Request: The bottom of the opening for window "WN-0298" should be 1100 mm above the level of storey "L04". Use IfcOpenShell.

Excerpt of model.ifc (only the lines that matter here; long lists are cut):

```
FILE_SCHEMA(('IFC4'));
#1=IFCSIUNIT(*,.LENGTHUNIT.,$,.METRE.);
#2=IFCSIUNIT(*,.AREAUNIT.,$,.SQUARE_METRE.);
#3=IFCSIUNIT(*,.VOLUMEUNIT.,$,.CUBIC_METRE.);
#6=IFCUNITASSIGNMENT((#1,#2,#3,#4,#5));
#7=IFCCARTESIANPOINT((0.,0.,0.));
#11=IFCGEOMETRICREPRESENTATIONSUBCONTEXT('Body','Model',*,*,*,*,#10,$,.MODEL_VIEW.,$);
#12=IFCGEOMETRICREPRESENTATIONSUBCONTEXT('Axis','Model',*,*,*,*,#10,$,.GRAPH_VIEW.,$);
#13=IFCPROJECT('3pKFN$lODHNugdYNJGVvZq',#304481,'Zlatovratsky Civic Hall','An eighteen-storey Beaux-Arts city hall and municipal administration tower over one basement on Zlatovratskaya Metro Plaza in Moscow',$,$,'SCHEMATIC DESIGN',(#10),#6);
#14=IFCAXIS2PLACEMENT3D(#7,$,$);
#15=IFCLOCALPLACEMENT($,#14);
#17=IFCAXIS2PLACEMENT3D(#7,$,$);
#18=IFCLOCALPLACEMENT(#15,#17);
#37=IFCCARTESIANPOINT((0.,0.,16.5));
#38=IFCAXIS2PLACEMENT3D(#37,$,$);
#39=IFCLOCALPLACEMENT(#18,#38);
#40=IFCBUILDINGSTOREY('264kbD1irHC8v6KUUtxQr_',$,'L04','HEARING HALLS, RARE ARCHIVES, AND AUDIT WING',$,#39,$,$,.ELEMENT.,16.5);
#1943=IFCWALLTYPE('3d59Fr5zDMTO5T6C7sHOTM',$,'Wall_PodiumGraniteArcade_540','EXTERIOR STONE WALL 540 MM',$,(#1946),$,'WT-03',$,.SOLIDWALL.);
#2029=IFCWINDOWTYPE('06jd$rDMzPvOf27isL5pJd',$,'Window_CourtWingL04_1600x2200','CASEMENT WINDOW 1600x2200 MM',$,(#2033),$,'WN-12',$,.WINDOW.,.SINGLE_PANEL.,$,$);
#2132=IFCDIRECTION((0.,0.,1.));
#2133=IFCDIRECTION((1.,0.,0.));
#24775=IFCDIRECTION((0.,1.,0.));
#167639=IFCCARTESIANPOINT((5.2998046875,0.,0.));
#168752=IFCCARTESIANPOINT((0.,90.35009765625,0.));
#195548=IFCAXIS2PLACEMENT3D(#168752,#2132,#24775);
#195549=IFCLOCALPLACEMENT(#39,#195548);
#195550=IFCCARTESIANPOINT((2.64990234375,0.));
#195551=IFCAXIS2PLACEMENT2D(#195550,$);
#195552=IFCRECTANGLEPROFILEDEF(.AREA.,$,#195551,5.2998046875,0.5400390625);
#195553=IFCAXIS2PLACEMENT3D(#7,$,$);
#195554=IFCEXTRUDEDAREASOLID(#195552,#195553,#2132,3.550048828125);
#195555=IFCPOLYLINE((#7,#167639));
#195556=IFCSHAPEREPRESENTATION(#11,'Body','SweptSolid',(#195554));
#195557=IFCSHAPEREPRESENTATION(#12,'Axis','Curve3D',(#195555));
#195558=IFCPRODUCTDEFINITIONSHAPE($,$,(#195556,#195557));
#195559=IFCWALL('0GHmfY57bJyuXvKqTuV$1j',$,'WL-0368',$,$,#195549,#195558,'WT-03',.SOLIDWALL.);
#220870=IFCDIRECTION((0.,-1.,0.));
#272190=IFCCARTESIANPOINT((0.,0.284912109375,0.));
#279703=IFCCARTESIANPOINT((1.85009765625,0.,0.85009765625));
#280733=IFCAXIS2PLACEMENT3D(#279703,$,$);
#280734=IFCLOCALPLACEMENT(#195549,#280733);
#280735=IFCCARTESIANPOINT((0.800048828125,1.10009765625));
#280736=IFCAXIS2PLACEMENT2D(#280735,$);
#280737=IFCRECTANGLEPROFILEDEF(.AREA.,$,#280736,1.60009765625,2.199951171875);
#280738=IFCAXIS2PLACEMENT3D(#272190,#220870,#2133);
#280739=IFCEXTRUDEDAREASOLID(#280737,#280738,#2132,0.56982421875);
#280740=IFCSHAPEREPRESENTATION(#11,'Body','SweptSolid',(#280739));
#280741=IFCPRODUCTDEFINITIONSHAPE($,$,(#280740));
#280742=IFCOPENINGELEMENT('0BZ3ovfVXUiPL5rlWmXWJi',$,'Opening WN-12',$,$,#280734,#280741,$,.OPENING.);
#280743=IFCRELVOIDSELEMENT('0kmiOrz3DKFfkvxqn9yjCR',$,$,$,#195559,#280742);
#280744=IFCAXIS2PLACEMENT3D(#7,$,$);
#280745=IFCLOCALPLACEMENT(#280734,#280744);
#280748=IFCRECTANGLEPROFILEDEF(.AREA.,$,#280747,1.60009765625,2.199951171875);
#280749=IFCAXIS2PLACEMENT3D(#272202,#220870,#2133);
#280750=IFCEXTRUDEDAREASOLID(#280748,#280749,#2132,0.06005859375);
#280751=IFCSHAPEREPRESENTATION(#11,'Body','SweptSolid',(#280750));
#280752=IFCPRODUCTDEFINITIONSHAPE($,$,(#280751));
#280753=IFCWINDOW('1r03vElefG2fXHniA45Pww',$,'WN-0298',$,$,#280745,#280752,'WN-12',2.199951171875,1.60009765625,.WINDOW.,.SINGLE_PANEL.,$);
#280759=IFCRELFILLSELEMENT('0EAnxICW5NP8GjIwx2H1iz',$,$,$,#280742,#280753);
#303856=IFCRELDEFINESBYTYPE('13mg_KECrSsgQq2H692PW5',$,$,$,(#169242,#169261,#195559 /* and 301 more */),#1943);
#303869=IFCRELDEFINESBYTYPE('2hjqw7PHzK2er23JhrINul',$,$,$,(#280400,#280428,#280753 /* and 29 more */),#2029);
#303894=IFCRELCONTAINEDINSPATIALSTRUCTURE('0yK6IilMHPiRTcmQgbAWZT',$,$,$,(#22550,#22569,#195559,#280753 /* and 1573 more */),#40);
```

```python
import numpy as np
import ifcopenshell
import ifcopenshell.api.geometry
import ifcopenshell.geom
import ifcopenshell.util.element
import ifcopenshell.util.placement
import ifcopenshell.util.shape
import ifcopenshell.util.unit

model = ifcopenshell.open("model.ifc")
unit_scale = ifcopenshell.util.unit.calculate_unit_scale(model)

window = model.by_guid("1r03vElefG2fXHniA45Pww")
opening = window.FillsVoids[0].RelatingOpeningElement
storey = ifcopenshell.util.element.get_container(window, ifc_class="IfcBuildingStorey")
level = ifcopenshell.util.placement.get_local_placement(storey.ObjectPlacement)[2, 3]

# The opening's origin need not be at the sill, so measure its lowest point.
shape = ifcopenshell.geom.create_shape(ifcopenshell.geom.settings(), opening)
bottom = ifcopenshell.util.shape.get_shape_bottom_elevation(shape, shape.geometry) / unit_scale
dz = level + 1.1 - bottom

shift = np.array([0.0, 0.0, dz])
# The window is placed relative to its opening, so it follows when the opening moves.
matrix = ifcopenshell.util.placement.get_local_placement(opening.ObjectPlacement)
matrix[:3, 3] += shift
ifcopenshell.api.geometry.edit_object_placement(
    model, product=opening, matrix=matrix, is_si=False, should_transform_children=True
)

print(f"moved by {dz * unit_scale:+.3f} m")

model.write("model_edited.ifc")
```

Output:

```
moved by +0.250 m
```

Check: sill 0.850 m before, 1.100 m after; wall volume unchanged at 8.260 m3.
